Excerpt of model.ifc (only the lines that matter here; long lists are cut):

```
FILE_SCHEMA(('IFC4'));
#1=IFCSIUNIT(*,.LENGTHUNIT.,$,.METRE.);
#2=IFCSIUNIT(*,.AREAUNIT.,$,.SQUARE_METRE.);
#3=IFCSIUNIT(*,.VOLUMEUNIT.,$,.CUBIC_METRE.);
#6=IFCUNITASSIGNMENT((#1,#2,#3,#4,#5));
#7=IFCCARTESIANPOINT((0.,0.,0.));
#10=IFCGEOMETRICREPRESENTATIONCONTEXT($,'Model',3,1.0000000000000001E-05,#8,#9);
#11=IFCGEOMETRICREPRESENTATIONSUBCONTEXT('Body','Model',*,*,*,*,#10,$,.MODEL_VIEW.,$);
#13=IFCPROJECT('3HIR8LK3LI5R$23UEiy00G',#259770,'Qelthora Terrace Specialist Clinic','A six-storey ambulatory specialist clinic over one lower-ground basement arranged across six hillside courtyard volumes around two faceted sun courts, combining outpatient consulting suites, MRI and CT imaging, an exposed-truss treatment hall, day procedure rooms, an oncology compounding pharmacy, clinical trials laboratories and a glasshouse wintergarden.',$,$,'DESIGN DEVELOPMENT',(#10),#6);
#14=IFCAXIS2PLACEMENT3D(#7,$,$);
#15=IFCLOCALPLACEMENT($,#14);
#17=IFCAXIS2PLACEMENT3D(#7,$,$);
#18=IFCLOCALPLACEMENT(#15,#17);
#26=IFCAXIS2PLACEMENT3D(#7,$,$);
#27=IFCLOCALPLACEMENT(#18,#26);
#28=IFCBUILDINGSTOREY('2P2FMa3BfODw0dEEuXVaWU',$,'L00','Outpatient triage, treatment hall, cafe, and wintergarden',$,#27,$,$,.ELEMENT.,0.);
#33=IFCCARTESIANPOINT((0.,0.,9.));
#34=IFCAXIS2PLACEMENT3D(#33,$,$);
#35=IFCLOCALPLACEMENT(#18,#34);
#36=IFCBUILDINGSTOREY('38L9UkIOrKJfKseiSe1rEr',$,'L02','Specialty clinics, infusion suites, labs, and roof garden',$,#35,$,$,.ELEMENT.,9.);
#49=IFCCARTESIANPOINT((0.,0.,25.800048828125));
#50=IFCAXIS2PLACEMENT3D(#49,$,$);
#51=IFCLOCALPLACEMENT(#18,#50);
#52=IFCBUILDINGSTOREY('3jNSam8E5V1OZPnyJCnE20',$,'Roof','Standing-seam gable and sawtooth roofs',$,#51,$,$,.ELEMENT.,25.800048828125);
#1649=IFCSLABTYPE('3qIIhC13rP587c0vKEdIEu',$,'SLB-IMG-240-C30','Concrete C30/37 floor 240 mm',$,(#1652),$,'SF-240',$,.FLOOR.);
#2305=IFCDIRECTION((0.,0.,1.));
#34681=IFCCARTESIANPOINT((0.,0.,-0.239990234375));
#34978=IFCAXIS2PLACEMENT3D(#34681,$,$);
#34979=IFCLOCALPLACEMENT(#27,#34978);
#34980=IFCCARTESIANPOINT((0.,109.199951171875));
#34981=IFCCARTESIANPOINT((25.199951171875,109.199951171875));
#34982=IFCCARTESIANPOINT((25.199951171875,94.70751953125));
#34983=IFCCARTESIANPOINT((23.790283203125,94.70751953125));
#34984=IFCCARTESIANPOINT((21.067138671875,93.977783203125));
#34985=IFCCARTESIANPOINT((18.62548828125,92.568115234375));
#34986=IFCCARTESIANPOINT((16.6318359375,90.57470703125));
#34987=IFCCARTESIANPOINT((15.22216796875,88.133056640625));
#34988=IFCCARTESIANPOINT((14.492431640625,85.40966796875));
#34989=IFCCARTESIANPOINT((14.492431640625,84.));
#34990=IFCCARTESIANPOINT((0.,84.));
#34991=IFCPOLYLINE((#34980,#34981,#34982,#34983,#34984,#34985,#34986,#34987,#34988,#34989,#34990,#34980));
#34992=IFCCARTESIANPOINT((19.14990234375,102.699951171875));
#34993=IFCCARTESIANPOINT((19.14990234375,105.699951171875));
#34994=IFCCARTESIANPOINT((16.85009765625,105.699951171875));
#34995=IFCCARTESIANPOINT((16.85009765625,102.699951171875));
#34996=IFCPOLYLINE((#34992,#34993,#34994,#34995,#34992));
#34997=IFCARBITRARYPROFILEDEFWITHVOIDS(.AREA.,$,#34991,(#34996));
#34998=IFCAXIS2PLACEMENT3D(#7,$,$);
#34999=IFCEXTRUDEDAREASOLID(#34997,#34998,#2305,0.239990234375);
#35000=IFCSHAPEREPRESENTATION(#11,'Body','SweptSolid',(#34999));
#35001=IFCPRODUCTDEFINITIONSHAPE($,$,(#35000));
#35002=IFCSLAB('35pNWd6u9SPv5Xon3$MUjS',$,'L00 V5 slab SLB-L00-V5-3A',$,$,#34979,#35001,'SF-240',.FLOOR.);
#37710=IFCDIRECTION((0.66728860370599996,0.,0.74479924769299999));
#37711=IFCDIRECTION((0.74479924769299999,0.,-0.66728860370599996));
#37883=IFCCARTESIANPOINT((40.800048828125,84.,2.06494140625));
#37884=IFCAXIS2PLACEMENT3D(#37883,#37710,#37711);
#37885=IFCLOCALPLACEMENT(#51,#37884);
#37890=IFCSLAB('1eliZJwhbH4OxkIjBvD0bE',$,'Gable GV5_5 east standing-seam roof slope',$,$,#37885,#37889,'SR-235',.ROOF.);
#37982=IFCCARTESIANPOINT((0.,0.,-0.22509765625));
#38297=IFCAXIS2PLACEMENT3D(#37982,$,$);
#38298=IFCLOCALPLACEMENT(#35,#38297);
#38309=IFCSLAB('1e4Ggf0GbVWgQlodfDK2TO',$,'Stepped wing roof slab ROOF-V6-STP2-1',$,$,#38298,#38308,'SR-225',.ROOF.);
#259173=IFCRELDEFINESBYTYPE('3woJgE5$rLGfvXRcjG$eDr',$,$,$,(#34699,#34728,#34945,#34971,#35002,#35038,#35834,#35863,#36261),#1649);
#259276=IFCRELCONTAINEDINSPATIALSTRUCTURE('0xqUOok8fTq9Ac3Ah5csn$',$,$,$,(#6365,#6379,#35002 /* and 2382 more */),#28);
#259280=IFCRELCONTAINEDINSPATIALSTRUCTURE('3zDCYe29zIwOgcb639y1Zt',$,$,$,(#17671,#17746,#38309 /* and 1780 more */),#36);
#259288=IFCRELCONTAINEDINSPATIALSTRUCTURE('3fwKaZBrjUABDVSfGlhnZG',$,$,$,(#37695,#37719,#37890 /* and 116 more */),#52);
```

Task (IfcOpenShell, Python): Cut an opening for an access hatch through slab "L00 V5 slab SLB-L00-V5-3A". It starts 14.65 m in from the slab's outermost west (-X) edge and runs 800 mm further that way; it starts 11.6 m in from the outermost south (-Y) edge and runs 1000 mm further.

```python
import numpy as np
import ifcopenshell
import ifcopenshell.api.feature
import ifcopenshell.api.geometry
import ifcopenshell.api.root
import ifcopenshell.geom
import ifcopenshell.util.placement
import ifcopenshell.util.representation
import ifcopenshell.util.shape
import ifcopenshell.util.unit

model = ifcopenshell.open("model.ifc")
unit_scale = ifcopenshell.util.unit.calculate_unit_scale(model)
settings = ifcopenshell.geom.settings()


def volume(element):
    """Net volume in cubic metres, openings subtracted."""
    shape = ifcopenshell.geom.create_shape(settings, element)
    return ifcopenshell.util.shape.get_volume(shape.geometry)


slab = model.by_guid("35pNWd6u9SPv5Xon3$MUjS")
before = volume(slab)

# Extent in the slab's own axes, in metres. The edges named are its -X and -Y sides.
slab_shape = ifcopenshell.geom.create_shape(settings, slab)
vertices = ifcopenshell.util.shape.get_vertices(slab_shape.geometry)
x_min, y_min, bottom = vertices.min(axis=0)
top = vertices[:, 2].max()

opening = ifcopenshell.api.root.create_entity(model, ifc_class="IfcOpeningElement", name="Access hatch opening", predefined_type="OPENING")
context = ifcopenshell.util.representation.get_context(model, "Model", "Body", "MODEL_VIEW")
width, depth = 0.8, 1
outline = [(0.0, 0.0), (width, 0.0), (width, depth), (0.0, depth), (0.0, 0.0)]
# Overshoot both faces by 50 mm so the cut is clean.
shape = ifcopenshell.api.geometry.add_slab_representation(
    model, context=context, depth=top - bottom + 0.1, polyline=outline
)
ifcopenshell.api.geometry.assign_representation(model, product=opening, representation=shape)

matrix = ifcopenshell.util.placement.get_local_placement(slab.ObjectPlacement)
matrix[:, 3] = matrix @ np.append(np.array([x_min + 14.65, y_min + 11.6, bottom - 0.05]) / unit_scale, 1.0)
ifcopenshell.api.geometry.edit_object_placement(model, product=opening, matrix=matrix, is_si=False)
ifcopenshell.api.feature.add_feature(model, feature=opening, element=slab)

after = volume(slab)

print(f"slab volume {before:.3f} -> {after:.3f} m3")

model.write("model_v2.ifc")
```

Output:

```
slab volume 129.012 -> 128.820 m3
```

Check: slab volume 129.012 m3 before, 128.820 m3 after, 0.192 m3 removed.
